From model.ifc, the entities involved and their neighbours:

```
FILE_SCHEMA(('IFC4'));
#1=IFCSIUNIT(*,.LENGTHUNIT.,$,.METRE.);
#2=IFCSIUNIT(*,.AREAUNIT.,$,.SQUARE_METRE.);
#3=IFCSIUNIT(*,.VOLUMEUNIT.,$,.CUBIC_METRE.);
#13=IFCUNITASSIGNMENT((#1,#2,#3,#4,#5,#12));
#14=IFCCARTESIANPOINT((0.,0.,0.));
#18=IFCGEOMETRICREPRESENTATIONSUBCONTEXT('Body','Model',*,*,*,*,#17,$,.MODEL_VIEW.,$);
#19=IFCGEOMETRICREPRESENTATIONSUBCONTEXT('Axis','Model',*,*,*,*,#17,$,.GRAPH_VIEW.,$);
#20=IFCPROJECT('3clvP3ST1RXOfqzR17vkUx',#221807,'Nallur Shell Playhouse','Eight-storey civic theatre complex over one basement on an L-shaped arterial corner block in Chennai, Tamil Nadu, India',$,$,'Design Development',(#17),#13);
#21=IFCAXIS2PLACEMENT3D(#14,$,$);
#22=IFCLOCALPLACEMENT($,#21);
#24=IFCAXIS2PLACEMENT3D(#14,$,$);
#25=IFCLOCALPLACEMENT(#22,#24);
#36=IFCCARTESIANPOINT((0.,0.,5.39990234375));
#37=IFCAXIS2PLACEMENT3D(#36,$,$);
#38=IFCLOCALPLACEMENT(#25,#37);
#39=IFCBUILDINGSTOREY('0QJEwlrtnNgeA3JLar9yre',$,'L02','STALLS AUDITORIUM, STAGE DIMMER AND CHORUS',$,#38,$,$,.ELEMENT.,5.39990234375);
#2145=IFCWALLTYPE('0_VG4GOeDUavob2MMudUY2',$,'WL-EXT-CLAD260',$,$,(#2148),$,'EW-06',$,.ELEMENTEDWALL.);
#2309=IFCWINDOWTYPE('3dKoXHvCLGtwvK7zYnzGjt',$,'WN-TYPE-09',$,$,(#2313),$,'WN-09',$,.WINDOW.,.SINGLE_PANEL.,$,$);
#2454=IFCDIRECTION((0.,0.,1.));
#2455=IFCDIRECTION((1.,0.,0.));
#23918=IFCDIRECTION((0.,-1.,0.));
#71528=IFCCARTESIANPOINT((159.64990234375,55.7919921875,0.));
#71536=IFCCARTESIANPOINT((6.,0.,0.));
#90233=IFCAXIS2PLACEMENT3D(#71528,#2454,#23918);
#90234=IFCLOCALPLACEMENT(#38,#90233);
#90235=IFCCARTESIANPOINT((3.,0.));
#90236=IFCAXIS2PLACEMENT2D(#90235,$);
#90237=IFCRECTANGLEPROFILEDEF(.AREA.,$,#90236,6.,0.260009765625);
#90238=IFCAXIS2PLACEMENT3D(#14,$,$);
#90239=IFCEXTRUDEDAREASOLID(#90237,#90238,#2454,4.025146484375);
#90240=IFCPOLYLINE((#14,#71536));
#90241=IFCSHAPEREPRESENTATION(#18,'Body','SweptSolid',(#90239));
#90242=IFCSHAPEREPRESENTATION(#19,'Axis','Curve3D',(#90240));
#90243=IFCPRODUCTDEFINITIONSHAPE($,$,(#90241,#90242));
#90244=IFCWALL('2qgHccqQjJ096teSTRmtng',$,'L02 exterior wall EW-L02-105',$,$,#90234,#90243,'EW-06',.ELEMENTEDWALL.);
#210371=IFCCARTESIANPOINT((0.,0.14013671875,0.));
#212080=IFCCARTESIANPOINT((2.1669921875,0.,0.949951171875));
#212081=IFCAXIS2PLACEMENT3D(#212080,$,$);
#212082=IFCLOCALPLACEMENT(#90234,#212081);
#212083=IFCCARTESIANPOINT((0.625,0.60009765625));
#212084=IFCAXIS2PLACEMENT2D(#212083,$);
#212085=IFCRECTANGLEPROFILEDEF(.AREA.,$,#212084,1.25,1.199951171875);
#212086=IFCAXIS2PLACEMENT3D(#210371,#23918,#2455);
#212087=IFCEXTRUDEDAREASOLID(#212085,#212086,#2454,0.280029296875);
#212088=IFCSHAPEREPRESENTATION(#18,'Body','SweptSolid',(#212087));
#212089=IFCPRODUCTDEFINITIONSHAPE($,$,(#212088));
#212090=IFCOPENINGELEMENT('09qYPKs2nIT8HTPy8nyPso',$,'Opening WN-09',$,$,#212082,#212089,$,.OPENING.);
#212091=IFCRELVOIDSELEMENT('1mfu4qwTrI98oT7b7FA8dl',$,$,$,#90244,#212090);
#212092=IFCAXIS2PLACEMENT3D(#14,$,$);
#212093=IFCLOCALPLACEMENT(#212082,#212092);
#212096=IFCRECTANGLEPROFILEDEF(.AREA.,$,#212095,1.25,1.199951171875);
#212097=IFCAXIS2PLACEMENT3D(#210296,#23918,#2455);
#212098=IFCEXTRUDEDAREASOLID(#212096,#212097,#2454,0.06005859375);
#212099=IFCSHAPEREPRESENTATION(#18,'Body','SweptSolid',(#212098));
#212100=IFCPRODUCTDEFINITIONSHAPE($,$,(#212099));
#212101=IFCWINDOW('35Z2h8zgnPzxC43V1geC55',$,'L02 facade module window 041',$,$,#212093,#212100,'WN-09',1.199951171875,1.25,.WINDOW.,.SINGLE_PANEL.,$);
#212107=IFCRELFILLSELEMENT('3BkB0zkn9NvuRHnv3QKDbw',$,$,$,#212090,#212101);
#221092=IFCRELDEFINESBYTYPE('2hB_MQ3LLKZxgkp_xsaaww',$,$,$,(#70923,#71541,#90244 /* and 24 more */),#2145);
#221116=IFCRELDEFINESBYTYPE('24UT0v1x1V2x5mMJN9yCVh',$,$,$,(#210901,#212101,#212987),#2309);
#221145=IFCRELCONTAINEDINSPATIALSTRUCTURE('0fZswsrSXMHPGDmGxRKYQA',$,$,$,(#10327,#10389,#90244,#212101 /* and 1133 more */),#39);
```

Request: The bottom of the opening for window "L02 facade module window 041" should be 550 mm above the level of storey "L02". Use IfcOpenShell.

```python
import numpy as np
import ifcopenshell
import ifcopenshell.api.geometry
import ifcopenshell.geom
import ifcopenshell.util.element
import ifcopenshell.util.placement
import ifcopenshell.util.shape
import ifcopenshell.util.unit

model = ifcopenshell.open("model.ifc")
unit_scale = ifcopenshell.util.unit.calculate_unit_scale(model)

window = model.by_id(212101)
opening = window.FillsVoids[0].RelatingOpeningElement
storey = ifcopenshell.util.element.get_container(window, ifc_class="IfcBuildingStorey")
level = ifcopenshell.util.placement.get_local_placement(storey.ObjectPlacement)[2, 3]

# The opening's origin need not be at the sill, so measure its lowest point.
shape = ifcopenshell.geom.create_shape(ifcopenshell.geom.settings(), opening)
bottom = ifcopenshell.util.shape.get_shape_bottom_elevation(shape, shape.geometry) / unit_scale
dz = level + 0.55 / unit_scale - bottom

shift = np.array([0.0, 0.0, dz])
# The window is placed relative to its opening, so it follows when the opening moves.
matrix = ifcopenshell.util.placement.get_local_placement(opening.ObjectPlacement)
matrix[:3, 3] += shift
ifcopenshell.api.geometry.edit_object_placement(
    model, product=opening, matrix=matrix, is_si=False, should_transform_children=True
)

print(f"moved by {dz * unit_scale:+.3f} m")

model.write("model_v2.ifc")
```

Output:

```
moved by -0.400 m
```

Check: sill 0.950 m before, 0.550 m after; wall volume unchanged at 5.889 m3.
